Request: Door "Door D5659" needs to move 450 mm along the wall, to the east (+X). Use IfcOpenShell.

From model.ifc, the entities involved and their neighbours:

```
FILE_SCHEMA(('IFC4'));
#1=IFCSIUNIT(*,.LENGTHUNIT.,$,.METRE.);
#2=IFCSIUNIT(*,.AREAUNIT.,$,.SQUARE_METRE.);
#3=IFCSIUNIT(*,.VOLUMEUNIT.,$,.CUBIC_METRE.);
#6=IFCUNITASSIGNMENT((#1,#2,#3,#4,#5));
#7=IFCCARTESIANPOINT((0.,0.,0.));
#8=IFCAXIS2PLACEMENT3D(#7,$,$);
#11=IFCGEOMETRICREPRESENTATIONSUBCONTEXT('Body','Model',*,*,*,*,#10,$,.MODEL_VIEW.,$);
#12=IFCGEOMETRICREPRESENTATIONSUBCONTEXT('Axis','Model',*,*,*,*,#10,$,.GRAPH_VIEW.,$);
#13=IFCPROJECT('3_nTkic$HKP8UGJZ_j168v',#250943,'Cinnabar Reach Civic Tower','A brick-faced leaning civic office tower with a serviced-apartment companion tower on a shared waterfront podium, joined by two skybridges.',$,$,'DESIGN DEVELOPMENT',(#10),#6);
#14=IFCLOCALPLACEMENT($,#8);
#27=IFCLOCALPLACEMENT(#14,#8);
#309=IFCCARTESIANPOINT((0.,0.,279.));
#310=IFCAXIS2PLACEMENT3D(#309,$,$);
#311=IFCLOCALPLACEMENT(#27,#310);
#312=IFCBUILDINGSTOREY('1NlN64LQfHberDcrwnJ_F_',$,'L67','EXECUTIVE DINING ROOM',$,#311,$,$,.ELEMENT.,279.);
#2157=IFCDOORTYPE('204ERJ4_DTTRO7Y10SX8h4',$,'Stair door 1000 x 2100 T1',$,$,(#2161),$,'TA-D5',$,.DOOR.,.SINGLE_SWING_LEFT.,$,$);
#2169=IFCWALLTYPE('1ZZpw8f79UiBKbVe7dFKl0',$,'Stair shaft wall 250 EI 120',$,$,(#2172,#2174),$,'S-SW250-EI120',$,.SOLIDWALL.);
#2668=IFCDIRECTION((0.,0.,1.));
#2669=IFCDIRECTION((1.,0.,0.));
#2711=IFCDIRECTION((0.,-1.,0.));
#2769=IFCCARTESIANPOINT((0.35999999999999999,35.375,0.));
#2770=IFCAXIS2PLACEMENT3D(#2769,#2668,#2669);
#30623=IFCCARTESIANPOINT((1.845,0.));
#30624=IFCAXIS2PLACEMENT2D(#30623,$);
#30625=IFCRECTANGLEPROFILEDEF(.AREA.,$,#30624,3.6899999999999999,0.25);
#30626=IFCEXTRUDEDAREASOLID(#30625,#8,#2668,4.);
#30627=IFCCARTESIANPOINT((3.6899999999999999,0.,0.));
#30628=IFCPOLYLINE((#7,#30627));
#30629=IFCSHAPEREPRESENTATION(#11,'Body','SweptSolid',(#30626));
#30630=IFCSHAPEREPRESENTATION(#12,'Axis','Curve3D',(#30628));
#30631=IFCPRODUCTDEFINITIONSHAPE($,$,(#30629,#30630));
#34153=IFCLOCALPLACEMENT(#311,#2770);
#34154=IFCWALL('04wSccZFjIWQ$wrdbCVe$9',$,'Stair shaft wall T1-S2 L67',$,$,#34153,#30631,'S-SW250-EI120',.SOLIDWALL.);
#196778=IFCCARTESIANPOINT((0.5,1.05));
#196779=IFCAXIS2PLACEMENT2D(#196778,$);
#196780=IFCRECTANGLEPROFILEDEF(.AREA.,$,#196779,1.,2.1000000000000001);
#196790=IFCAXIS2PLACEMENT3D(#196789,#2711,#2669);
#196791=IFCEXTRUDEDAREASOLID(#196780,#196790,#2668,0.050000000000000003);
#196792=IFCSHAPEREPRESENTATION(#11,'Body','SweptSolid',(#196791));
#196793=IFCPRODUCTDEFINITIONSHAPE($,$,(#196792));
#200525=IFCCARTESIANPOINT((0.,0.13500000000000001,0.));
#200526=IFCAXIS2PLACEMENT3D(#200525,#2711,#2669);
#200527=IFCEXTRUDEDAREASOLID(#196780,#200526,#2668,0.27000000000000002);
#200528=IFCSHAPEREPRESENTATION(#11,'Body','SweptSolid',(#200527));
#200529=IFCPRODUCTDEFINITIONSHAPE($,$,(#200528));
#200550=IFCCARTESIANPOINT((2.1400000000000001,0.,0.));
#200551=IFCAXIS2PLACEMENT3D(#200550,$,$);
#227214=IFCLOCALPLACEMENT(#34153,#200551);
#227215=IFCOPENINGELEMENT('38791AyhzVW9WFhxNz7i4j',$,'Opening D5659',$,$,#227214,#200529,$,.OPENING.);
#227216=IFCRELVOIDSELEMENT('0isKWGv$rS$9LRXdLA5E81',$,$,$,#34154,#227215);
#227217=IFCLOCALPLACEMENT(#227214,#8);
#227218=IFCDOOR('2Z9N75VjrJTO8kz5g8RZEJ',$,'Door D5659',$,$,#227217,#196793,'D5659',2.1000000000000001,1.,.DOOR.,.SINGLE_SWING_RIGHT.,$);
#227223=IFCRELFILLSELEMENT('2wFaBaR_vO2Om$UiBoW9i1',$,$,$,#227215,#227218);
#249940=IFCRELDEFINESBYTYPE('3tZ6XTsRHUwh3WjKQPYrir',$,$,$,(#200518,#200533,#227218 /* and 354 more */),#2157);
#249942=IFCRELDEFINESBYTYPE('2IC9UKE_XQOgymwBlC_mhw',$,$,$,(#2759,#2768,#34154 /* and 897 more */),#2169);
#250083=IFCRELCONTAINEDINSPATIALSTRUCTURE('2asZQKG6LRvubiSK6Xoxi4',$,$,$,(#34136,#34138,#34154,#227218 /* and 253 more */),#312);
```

```python
import ifcopenshell
import ifcopenshell.api.geometry
import ifcopenshell.util.placement

model = ifcopenshell.open("model.ifc")

door = model.by_id(227218)
opening = door.FillsVoids[0].RelatingOpeningElement
wall = opening.VoidsElements[0].RelatingBuildingElement

wall_matrix = ifcopenshell.util.placement.get_local_placement(wall.ObjectPlacement)
shift = wall_matrix[:3, 0] * 0.45
before = ifcopenshell.util.placement.get_local_placement(door.ObjectPlacement)[:3, 3].copy()

# The door is placed relative to its opening, so it follows when the opening moves.
matrix = ifcopenshell.util.placement.get_local_placement(opening.ObjectPlacement)
matrix[:3, 3] += shift
ifcopenshell.api.geometry.edit_object_placement(
    model, product=opening, matrix=matrix, is_si=False, should_transform_children=True
)

after = ifcopenshell.util.placement.get_local_placement(door.ObjectPlacement)[:3, 3]
print("door moved by", (after - before).round(3) + 0.0)

model.write("model-out.ifc")
```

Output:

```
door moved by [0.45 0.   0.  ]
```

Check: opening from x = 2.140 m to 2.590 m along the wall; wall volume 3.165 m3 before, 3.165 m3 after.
